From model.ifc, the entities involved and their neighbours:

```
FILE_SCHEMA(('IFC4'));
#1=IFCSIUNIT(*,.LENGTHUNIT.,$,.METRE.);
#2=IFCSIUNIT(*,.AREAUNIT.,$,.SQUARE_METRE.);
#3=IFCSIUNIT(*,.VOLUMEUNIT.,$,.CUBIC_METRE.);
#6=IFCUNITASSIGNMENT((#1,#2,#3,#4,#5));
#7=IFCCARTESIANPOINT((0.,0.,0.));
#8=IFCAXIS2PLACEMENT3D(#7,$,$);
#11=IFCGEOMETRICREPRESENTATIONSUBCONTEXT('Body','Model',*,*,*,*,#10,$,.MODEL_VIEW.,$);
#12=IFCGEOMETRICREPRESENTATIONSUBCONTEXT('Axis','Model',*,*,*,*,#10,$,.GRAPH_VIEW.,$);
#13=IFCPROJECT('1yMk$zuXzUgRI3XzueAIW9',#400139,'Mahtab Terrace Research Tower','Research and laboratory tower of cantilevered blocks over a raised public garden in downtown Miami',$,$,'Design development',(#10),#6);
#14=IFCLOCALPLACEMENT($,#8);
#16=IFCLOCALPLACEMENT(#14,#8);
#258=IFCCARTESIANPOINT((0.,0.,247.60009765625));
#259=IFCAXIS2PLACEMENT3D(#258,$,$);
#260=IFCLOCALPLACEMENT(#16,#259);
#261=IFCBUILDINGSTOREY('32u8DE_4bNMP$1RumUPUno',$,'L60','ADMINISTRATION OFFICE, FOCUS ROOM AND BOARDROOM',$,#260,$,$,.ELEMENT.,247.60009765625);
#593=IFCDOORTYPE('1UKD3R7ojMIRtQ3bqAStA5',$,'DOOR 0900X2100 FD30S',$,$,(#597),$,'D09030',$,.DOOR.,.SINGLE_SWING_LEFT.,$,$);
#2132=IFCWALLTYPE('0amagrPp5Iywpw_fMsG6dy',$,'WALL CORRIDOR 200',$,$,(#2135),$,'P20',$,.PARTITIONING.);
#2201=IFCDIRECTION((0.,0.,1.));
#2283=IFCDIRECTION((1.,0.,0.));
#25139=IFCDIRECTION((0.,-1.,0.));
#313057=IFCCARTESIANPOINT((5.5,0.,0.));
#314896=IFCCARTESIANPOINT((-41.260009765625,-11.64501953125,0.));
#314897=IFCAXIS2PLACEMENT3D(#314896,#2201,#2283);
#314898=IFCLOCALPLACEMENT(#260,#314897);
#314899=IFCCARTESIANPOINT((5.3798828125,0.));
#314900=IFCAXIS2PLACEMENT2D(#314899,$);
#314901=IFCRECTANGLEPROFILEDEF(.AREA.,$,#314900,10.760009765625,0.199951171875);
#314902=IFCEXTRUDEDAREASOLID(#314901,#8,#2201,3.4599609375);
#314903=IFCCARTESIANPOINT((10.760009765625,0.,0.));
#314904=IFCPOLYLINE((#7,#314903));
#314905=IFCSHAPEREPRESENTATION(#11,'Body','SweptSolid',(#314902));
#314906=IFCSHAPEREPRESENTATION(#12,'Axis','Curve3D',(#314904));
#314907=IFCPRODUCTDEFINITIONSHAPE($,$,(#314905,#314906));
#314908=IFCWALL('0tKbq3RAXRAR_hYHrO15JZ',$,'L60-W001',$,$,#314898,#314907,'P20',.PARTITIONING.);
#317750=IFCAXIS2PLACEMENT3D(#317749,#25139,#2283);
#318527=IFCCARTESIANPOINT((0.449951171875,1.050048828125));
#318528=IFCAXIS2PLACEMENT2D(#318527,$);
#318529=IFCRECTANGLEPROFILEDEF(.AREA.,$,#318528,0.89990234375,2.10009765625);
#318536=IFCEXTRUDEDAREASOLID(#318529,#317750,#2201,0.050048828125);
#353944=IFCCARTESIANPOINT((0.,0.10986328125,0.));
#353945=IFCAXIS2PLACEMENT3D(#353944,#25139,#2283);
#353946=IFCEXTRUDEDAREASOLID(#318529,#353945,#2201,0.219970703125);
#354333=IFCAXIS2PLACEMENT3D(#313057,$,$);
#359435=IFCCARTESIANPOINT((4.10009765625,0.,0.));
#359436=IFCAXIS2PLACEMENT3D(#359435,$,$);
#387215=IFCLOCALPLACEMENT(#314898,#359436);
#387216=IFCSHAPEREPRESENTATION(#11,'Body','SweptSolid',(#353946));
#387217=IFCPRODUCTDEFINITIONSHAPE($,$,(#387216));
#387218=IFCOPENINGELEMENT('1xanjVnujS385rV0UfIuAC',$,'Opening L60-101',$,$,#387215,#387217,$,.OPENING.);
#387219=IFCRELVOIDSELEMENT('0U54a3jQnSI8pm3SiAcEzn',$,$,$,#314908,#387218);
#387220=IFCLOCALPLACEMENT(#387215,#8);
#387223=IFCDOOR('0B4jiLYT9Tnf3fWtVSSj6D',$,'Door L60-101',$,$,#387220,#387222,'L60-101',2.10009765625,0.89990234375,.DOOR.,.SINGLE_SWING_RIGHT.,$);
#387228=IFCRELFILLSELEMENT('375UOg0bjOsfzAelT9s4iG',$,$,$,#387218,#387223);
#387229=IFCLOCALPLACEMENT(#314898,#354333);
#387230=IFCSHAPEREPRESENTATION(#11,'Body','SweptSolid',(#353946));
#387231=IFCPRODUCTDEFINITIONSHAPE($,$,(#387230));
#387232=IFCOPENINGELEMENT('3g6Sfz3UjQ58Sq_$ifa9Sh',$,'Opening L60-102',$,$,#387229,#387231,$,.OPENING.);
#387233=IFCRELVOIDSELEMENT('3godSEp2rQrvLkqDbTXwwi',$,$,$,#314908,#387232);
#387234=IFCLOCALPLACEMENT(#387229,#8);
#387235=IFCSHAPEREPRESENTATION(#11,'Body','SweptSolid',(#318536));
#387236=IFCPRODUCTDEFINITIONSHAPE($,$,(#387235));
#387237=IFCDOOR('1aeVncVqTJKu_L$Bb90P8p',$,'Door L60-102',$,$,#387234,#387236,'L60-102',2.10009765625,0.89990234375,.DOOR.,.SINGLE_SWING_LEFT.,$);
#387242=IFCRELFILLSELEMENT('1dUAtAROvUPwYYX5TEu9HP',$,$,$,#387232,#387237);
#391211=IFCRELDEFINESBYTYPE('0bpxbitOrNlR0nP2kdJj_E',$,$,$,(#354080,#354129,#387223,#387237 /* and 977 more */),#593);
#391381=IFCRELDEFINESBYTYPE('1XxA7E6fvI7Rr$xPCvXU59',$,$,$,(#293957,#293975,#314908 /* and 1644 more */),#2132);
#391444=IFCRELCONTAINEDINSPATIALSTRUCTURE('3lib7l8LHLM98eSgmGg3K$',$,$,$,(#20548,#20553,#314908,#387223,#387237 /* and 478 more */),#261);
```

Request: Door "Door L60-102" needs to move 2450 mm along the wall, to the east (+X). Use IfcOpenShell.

```python
import ifcopenshell
import ifcopenshell.api.geometry
import ifcopenshell.util.placement

model = ifcopenshell.open("model.ifc")

door = model.by_id(387237)
opening = door.FillsVoids[0].RelatingOpeningElement
wall = opening.VoidsElements[0].RelatingBuildingElement

wall_matrix = ifcopenshell.util.placement.get_local_placement(wall.ObjectPlacement)
shift = wall_matrix[:3, 0] * 2.45
before = ifcopenshell.util.placement.get_local_placement(door.ObjectPlacement)[:3, 3].copy()

# The door is placed relative to its opening, so it follows when the opening moves.
matrix = ifcopenshell.util.placement.get_local_placement(opening.ObjectPlacement)
matrix[:3, 3] += shift
ifcopenshell.api.geometry.edit_object_placement(
    model, product=opening, matrix=matrix, is_si=False, should_transform_children=True
)

after = ifcopenshell.util.placement.get_local_placement(door.ObjectPlacement)[:3, 3]
print("door moved by", (after - before).round(3) + 0.0)

model.write("model_v2.ifc")
```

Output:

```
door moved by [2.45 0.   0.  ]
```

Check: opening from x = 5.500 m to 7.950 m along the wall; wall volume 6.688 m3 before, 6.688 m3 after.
